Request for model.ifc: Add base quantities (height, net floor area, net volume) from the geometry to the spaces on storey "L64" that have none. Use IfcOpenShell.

First a look at what the model holds.

```python
import ifcopenshell
import ifcopenshell.util.element
import ifcopenshell.util.unit

model = ifcopenshell.open("model.ifc")
print(model.schema)
for unit_type in ("LENGTHUNIT", "AREAUNIT", "VOLUMEUNIT"):
    print(unit_type, ifcopenshell.util.unit.calculate_unit_scale(model, unit_type))
storey = next(s for s in model.by_type("IfcBuildingStorey") if s.Name == "L64")
spaces = [e for e in ifcopenshell.util.element.get_decomposition(storey) if e.is_a("IfcSpace")]
for e in sorted(spaces, key=lambda e: e.id()):
    print(e.id(), e.is_a(), e.Name, list(ifcopenshell.util.element.get_psets(e, qtos_only=True)), sep=" | ")
```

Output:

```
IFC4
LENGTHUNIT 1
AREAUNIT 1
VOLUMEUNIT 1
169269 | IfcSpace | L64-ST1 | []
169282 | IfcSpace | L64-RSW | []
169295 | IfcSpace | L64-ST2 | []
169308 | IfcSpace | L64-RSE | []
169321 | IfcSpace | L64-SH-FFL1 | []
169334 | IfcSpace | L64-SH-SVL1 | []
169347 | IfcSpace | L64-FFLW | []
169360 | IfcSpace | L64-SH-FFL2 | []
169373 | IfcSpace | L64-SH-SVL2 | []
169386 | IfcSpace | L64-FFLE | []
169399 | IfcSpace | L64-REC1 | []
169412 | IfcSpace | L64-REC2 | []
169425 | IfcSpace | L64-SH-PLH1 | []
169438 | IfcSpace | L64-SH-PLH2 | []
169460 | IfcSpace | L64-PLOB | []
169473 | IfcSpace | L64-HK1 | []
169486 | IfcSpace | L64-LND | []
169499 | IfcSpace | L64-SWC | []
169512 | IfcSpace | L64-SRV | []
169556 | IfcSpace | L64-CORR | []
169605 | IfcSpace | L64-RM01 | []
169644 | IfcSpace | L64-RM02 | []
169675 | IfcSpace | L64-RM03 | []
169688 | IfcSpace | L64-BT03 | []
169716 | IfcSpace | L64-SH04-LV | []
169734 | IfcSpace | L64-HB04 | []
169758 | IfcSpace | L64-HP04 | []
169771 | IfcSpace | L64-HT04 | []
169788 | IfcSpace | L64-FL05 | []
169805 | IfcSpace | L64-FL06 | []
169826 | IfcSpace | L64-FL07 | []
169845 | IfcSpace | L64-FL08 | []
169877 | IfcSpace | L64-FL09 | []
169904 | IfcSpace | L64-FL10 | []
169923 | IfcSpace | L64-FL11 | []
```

```python
import ifcopenshell
import ifcopenshell.api.pset
import ifcopenshell.geom
import ifcopenshell.util.element
import ifcopenshell.util.shape
import ifcopenshell.util.unit

model = ifcopenshell.open("model.ifc")
unit_scale = ifcopenshell.util.unit.calculate_unit_scale(model)
area_scale = ifcopenshell.util.unit.calculate_unit_scale(model, "AREAUNIT")
volume_scale = ifcopenshell.util.unit.calculate_unit_scale(model, "VOLUMEUNIT")
settings = ifcopenshell.geom.settings()

storey = next(s for s in model.by_type("IfcBuildingStorey") if s.Name == "L64")
spaces = [e for e in ifcopenshell.util.element.get_decomposition(storey) if e.is_a("IfcSpace")]

for e in sorted(spaces, key=lambda e: e.id()):
    if ifcopenshell.util.element.get_psets(e, qtos_only=True, should_inherit=False):
        continue
    # Geometry comes back in metres, in the element's own axes.
    shape = ifcopenshell.geom.create_shape(settings, e)
    values = {
        "Height": ifcopenshell.util.shape.get_z(shape.geometry) / unit_scale,
        "NetFloorArea": ifcopenshell.util.shape.get_footprint_area(shape.geometry) / area_scale,
        "NetVolume": ifcopenshell.util.shape.get_volume(shape.geometry) / volume_scale,
    }
    qto = ifcopenshell.api.pset.add_qto(model, product=e, name="Qto_SpaceBaseQuantities")
    ifcopenshell.api.pset.edit_qto(model, qto=qto, properties=values)
    print(e.id(), {k: round(v, 3) for k, v in values.items()})

model.write("model_v2.ifc")
```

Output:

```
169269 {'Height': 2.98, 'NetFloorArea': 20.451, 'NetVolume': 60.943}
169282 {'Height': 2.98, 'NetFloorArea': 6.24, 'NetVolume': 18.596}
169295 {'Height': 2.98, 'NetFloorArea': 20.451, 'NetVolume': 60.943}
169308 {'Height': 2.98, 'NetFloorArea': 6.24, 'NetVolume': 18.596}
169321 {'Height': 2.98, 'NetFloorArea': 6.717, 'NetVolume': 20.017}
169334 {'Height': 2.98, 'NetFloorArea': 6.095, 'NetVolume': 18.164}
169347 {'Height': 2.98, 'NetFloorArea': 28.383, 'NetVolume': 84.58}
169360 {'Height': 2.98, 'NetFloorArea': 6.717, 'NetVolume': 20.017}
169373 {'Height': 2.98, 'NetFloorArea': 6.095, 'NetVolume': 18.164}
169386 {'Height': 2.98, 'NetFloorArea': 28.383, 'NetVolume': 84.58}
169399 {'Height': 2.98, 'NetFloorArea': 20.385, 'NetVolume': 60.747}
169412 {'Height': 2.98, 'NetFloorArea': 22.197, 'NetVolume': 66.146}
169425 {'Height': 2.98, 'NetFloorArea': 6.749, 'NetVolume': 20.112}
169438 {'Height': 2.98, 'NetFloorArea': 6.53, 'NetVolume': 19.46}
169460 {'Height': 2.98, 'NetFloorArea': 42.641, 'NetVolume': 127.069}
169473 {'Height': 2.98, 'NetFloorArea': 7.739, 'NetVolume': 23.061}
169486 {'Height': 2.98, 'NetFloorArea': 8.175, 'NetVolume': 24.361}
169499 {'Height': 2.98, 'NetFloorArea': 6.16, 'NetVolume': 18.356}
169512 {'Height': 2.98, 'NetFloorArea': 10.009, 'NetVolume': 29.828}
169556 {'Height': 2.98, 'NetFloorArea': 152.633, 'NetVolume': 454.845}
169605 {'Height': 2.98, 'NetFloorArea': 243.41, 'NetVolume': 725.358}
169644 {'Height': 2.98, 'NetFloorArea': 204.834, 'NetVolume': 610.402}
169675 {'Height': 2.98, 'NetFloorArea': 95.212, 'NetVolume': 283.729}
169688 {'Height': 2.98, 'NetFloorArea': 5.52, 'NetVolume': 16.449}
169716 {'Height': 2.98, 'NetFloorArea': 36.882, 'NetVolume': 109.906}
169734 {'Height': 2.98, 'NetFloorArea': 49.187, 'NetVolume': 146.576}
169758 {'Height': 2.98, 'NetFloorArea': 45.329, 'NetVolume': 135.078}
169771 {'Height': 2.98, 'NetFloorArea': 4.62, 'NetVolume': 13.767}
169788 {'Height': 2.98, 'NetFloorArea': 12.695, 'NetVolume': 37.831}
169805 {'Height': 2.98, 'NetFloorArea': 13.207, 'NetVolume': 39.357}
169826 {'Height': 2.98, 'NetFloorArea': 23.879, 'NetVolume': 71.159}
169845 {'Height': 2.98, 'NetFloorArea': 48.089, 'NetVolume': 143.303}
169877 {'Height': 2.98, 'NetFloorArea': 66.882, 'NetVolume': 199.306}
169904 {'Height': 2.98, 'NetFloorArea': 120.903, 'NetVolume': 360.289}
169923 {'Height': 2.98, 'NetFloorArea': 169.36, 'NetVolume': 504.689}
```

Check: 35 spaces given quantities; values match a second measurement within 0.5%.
